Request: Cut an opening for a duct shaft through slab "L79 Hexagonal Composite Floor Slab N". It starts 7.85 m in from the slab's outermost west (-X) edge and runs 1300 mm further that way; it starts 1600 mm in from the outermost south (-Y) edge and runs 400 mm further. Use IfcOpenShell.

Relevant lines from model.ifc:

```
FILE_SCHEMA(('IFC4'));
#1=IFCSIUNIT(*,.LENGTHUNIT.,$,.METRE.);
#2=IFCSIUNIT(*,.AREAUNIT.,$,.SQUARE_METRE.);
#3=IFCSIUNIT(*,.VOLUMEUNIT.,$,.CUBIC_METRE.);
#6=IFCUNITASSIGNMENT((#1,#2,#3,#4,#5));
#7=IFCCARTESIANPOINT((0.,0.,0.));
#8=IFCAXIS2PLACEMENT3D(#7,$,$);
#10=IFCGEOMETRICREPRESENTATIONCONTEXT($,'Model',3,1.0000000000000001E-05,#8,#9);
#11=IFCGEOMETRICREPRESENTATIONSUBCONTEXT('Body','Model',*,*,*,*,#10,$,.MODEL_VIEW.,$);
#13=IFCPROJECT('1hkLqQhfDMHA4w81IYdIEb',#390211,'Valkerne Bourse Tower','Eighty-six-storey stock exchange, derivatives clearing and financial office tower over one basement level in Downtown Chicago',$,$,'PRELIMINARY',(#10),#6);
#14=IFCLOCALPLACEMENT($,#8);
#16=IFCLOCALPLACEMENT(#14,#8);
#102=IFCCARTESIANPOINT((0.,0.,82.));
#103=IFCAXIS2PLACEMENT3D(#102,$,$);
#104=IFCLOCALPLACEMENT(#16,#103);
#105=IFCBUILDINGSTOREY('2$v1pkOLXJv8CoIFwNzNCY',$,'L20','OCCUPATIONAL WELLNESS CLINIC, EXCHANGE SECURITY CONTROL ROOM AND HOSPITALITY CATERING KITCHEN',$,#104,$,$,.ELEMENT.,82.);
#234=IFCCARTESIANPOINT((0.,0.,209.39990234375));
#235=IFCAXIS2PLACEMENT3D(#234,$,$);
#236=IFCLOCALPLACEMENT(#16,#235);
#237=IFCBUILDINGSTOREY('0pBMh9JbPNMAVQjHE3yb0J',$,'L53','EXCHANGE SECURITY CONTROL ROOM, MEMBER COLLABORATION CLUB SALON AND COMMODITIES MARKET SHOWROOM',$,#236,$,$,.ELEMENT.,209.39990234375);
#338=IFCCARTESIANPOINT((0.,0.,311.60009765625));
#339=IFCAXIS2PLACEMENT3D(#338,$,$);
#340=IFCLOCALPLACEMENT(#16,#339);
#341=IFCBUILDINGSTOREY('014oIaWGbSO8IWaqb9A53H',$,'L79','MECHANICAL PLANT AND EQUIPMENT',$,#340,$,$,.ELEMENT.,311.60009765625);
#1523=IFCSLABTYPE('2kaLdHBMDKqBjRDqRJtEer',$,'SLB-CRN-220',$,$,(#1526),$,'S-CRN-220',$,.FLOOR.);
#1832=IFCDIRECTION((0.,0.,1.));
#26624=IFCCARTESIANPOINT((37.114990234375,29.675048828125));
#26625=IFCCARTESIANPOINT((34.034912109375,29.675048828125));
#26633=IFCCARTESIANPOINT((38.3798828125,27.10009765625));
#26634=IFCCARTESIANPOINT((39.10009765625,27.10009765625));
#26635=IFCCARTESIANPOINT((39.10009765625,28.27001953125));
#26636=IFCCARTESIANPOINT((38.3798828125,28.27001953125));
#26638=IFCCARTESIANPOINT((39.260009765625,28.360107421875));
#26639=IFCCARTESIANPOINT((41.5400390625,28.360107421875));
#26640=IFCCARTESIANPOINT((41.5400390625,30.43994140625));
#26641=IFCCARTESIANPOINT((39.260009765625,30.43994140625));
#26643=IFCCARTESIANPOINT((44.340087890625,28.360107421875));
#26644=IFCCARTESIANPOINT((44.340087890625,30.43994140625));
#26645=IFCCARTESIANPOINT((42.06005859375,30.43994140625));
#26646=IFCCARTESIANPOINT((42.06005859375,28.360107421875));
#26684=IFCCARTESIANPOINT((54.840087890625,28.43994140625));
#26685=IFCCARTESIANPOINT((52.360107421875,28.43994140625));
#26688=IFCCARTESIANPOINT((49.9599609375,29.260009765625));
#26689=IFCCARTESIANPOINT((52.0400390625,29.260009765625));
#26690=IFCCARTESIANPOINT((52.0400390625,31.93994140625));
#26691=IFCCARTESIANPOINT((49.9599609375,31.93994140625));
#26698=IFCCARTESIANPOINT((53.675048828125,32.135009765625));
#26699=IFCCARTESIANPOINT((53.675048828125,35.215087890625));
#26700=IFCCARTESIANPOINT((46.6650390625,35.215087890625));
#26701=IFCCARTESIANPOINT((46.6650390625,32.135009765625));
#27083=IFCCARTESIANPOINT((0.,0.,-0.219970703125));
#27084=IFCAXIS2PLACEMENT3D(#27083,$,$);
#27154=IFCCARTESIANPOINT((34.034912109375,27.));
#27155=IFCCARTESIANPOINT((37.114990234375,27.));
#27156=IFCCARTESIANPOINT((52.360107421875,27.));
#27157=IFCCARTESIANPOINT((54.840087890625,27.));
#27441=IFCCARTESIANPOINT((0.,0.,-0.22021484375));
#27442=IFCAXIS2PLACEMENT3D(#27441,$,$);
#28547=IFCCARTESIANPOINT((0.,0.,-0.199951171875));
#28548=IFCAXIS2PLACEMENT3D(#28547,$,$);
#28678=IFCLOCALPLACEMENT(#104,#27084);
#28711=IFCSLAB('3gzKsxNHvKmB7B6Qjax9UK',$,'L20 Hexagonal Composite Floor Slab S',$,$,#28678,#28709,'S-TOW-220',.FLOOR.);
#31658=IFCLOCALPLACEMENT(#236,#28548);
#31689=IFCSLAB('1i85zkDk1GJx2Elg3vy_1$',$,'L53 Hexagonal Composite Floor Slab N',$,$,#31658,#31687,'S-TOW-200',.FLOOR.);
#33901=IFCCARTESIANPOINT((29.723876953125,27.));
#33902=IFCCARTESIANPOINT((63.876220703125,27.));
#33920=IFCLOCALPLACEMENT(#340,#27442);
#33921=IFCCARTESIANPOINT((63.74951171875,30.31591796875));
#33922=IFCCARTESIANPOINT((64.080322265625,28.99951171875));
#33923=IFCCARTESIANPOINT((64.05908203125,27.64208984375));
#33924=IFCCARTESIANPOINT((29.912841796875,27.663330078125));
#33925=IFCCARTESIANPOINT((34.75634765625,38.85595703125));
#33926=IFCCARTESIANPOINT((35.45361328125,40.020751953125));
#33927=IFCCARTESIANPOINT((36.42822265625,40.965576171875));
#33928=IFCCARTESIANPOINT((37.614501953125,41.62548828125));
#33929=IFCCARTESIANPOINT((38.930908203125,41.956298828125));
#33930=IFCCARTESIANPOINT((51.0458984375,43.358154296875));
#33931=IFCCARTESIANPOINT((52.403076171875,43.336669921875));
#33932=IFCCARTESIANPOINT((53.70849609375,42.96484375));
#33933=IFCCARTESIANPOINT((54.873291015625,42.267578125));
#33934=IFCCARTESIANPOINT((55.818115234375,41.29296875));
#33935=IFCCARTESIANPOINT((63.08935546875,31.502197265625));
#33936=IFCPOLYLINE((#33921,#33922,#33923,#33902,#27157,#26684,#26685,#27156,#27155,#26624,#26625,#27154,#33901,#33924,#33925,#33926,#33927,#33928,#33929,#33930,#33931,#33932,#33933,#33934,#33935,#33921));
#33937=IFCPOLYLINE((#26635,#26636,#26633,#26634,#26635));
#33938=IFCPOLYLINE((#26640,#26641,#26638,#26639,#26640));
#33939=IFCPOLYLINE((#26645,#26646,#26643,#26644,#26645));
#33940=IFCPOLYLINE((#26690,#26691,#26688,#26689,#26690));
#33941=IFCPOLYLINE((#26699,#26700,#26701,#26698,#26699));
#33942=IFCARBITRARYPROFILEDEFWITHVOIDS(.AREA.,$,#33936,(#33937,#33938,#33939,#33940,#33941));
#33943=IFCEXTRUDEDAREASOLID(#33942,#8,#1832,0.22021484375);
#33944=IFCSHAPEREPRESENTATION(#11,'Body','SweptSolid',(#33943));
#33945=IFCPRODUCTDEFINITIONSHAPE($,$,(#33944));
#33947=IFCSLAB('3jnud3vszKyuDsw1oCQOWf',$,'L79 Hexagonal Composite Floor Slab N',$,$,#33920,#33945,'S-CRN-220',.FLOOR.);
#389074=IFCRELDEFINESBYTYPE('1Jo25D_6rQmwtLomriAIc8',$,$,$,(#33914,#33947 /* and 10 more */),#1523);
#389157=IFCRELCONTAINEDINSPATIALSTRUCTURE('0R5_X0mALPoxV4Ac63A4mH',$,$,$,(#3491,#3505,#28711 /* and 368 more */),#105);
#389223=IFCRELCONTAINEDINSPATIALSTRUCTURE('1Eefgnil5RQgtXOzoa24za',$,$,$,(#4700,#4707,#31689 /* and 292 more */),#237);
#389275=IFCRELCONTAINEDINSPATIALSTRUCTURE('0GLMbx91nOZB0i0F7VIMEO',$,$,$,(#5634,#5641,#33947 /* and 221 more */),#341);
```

```python
import numpy as np
import ifcopenshell
import ifcopenshell.api.feature
import ifcopenshell.api.geometry
import ifcopenshell.api.root
import ifcopenshell.geom
import ifcopenshell.util.placement
import ifcopenshell.util.representation
import ifcopenshell.util.shape
import ifcopenshell.util.unit

model = ifcopenshell.open("model.ifc")
unit_scale = ifcopenshell.util.unit.calculate_unit_scale(model)
settings = ifcopenshell.geom.settings()


def volume(element):
    """Net volume in cubic metres, openings subtracted."""
    shape = ifcopenshell.geom.create_shape(settings, element)
    return ifcopenshell.util.shape.get_volume(shape.geometry)


slab = model.by_id(33947)
before = volume(slab)

# Extent in the slab's own axes, in metres. The edges named are its -X and -Y sides.
slab_shape = ifcopenshell.geom.create_shape(settings, slab)
vertices = ifcopenshell.util.shape.get_vertices(slab_shape.geometry)
x_min, y_min, bottom = vertices.min(axis=0)
top = vertices[:, 2].max()

opening = ifcopenshell.api.root.create_entity(model, ifc_class="IfcOpeningElement", name="Duct shaft opening", predefined_type="OPENING")
context = ifcopenshell.util.representation.get_context(model, "Model", "Body", "MODEL_VIEW")
width, depth = 1.3, 0.4
outline = [(0.0, 0.0), (width, 0.0), (width, depth), (0.0, depth), (0.0, 0.0)]
# Overshoot both faces by 50 mm so the cut is clean.
shape = ifcopenshell.api.geometry.add_slab_representation(
    model, context=context, depth=top - bottom + 0.1, polyline=outline
)
ifcopenshell.api.geometry.assign_representation(model, product=opening, representation=shape)

matrix = ifcopenshell.util.placement.get_local_placement(slab.ObjectPlacement)
matrix[:, 3] = matrix @ np.append(np.array([x_min + 7.85, y_min + 1.6, bottom - 0.05]) / unit_scale, 1.0)
ifcopenshell.api.geometry.edit_object_placement(model, product=opening, matrix=matrix, is_si=False)
ifcopenshell.api.feature.add_feature(model, feature=opening, element=slab)

after = volume(slab)

print(f"slab volume {before:.3f} -> {after:.3f} m3")

model.write("model_rev.ifc")
```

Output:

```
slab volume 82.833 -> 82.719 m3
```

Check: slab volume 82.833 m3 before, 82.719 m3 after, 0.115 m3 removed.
